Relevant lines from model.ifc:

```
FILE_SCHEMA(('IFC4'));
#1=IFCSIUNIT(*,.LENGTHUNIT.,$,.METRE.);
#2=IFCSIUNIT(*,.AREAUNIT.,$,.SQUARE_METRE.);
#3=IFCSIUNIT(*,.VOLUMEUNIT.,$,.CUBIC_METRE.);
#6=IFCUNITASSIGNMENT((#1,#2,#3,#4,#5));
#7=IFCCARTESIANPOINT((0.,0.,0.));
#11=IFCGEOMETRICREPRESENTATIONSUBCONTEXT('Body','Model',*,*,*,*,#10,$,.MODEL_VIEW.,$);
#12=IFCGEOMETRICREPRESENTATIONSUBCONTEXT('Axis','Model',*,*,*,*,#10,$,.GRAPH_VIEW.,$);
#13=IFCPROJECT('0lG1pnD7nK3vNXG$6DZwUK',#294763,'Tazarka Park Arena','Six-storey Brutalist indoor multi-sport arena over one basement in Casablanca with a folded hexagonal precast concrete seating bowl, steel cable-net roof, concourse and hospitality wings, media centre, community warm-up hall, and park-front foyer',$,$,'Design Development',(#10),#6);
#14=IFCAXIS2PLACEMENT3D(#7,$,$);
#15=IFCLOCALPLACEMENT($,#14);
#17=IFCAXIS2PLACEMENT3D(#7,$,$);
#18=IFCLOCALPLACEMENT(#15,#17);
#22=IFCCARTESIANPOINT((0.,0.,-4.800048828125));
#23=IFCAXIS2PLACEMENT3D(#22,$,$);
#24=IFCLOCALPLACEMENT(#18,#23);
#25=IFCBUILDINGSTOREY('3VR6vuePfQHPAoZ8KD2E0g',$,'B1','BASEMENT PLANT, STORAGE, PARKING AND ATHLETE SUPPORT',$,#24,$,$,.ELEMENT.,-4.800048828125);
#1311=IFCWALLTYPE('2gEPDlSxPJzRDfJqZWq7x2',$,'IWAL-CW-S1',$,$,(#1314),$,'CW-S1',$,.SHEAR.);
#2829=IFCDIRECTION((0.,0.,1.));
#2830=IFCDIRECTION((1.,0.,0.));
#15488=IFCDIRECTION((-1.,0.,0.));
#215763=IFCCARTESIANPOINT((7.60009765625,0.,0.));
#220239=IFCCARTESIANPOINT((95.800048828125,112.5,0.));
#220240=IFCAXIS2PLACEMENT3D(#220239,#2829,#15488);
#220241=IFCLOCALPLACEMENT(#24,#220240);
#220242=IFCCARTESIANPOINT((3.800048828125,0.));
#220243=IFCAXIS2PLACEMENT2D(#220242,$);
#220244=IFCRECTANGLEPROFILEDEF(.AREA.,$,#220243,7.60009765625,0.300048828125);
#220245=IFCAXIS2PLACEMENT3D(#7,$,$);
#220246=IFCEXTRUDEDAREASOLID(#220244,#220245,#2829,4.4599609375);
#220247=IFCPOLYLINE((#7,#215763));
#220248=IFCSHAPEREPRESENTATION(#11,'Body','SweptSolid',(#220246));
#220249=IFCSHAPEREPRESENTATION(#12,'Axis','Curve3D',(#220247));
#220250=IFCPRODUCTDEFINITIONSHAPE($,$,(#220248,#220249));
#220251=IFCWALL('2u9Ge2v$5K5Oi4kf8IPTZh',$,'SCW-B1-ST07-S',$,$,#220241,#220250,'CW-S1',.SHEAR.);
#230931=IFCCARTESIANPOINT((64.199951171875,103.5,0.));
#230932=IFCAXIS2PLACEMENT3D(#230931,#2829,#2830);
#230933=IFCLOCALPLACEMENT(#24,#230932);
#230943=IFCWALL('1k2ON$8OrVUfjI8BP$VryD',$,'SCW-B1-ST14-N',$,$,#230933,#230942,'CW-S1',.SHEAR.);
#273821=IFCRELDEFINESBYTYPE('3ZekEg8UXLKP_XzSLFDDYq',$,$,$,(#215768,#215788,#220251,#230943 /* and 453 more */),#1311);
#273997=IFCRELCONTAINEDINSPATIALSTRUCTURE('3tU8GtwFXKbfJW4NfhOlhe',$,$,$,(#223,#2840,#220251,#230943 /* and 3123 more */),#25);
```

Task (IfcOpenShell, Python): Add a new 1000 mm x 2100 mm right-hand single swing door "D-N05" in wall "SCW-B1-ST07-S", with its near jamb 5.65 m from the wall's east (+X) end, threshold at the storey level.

```python
import numpy as np
import ifcopenshell
import ifcopenshell.api.feature
import ifcopenshell.api.geometry
import ifcopenshell.api.root
import ifcopenshell.api.spatial
import ifcopenshell.geom
import ifcopenshell.util.element
import ifcopenshell.util.placement
import ifcopenshell.util.representation
import ifcopenshell.util.shape
import ifcopenshell.util.unit

model = ifcopenshell.open("model.ifc")
unit_scale = ifcopenshell.util.unit.calculate_unit_scale(model)
settings = ifcopenshell.geom.settings()


def volume(element):
    """Net volume in cubic metres, openings subtracted."""
    shape = ifcopenshell.geom.create_shape(settings, element)
    return ifcopenshell.util.shape.get_volume(shape.geometry)


wall = model.by_guid("2u9Ge2v$5K5Oi4kf8IPTZh")
storey = ifcopenshell.util.element.get_container(wall, ifc_class="IfcBuildingStorey")
context = ifcopenshell.util.representation.get_context(model, "Model", "Body", "MODEL_VIEW")
before = volume(wall)

width, height, from_end, sill = 1, 2.1, 5.65, 0.0  # metres

# The wall runs along its own X axis, and the end named is its -X end.
wall_shape = ifcopenshell.geom.create_shape(settings, wall)
x, y, z = ifcopenshell.util.shape.get_vertices(wall_shape.geometry).T
start = x.min() + from_end
face, thickness = float(y.min()), float(y.max() - y.min())
wall_matrix = ifcopenshell.util.placement.get_local_placement(wall.ObjectPlacement)
level = ifcopenshell.util.placement.get_local_placement(storey.ObjectPlacement)[2, 3]


def in_wall(x, y):
    """Placement at x, y metres in the wall's axes, at sill height."""
    matrix = wall_matrix.copy()
    matrix[:, 3] = wall_matrix @ np.array([x / unit_scale, y / unit_scale, 0.0, 1.0])
    matrix[2, 3] = level + sill / unit_scale
    return matrix


# Opening: a box that overshoots both wall faces by 50 mm.
opening = ifcopenshell.api.root.create_entity(model, ifc_class="IfcOpeningElement", predefined_type="OPENING")
box = ifcopenshell.api.geometry.add_wall_representation(
    model, context=context, length=width, height=height, thickness=thickness + 0.1
)
ifcopenshell.api.geometry.assign_representation(model, product=opening, representation=box)
ifcopenshell.api.geometry.edit_object_placement(model, product=opening, matrix=in_wall(start, face - 0.05), is_si=False)
ifcopenshell.api.feature.add_feature(model, feature=opening, element=wall)

door = ifcopenshell.api.root.create_entity(model, ifc_class="IfcDoor", name="D-N05", predefined_type="DOOR")
door.OverallWidth, door.OverallHeight = width / unit_scale, height / unit_scale
door.OperationType = "SINGLE_SWING_RIGHT"
body = ifcopenshell.api.geometry.add_door_representation(
    model,
    context=context,
    overall_width=door.OverallWidth,
    overall_height=door.OverallHeight,
    operation_type="SINGLE_SWING_RIGHT",
    lining_properties={"LiningDepth": thickness / unit_scale, "ThresholdDepth": thickness / unit_scale},
)
ifcopenshell.api.geometry.assign_representation(model, product=door, representation=body)
ifcopenshell.api.spatial.assign_container(model, products=[door], relating_structure=storey)
ifcopenshell.api.feature.add_filling(model, opening=opening, element=door)

# The lining spans the wall, so the door starts at the wall face.
ifcopenshell.api.geometry.edit_object_placement(model, product=door, matrix=in_wall(start, face), is_si=False)

after = volume(wall)

print(f"wall volume {before:.3f} -> {after:.3f} m3")

model.write("model_edited.ifc")
```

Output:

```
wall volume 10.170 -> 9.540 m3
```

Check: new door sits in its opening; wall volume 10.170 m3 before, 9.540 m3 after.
